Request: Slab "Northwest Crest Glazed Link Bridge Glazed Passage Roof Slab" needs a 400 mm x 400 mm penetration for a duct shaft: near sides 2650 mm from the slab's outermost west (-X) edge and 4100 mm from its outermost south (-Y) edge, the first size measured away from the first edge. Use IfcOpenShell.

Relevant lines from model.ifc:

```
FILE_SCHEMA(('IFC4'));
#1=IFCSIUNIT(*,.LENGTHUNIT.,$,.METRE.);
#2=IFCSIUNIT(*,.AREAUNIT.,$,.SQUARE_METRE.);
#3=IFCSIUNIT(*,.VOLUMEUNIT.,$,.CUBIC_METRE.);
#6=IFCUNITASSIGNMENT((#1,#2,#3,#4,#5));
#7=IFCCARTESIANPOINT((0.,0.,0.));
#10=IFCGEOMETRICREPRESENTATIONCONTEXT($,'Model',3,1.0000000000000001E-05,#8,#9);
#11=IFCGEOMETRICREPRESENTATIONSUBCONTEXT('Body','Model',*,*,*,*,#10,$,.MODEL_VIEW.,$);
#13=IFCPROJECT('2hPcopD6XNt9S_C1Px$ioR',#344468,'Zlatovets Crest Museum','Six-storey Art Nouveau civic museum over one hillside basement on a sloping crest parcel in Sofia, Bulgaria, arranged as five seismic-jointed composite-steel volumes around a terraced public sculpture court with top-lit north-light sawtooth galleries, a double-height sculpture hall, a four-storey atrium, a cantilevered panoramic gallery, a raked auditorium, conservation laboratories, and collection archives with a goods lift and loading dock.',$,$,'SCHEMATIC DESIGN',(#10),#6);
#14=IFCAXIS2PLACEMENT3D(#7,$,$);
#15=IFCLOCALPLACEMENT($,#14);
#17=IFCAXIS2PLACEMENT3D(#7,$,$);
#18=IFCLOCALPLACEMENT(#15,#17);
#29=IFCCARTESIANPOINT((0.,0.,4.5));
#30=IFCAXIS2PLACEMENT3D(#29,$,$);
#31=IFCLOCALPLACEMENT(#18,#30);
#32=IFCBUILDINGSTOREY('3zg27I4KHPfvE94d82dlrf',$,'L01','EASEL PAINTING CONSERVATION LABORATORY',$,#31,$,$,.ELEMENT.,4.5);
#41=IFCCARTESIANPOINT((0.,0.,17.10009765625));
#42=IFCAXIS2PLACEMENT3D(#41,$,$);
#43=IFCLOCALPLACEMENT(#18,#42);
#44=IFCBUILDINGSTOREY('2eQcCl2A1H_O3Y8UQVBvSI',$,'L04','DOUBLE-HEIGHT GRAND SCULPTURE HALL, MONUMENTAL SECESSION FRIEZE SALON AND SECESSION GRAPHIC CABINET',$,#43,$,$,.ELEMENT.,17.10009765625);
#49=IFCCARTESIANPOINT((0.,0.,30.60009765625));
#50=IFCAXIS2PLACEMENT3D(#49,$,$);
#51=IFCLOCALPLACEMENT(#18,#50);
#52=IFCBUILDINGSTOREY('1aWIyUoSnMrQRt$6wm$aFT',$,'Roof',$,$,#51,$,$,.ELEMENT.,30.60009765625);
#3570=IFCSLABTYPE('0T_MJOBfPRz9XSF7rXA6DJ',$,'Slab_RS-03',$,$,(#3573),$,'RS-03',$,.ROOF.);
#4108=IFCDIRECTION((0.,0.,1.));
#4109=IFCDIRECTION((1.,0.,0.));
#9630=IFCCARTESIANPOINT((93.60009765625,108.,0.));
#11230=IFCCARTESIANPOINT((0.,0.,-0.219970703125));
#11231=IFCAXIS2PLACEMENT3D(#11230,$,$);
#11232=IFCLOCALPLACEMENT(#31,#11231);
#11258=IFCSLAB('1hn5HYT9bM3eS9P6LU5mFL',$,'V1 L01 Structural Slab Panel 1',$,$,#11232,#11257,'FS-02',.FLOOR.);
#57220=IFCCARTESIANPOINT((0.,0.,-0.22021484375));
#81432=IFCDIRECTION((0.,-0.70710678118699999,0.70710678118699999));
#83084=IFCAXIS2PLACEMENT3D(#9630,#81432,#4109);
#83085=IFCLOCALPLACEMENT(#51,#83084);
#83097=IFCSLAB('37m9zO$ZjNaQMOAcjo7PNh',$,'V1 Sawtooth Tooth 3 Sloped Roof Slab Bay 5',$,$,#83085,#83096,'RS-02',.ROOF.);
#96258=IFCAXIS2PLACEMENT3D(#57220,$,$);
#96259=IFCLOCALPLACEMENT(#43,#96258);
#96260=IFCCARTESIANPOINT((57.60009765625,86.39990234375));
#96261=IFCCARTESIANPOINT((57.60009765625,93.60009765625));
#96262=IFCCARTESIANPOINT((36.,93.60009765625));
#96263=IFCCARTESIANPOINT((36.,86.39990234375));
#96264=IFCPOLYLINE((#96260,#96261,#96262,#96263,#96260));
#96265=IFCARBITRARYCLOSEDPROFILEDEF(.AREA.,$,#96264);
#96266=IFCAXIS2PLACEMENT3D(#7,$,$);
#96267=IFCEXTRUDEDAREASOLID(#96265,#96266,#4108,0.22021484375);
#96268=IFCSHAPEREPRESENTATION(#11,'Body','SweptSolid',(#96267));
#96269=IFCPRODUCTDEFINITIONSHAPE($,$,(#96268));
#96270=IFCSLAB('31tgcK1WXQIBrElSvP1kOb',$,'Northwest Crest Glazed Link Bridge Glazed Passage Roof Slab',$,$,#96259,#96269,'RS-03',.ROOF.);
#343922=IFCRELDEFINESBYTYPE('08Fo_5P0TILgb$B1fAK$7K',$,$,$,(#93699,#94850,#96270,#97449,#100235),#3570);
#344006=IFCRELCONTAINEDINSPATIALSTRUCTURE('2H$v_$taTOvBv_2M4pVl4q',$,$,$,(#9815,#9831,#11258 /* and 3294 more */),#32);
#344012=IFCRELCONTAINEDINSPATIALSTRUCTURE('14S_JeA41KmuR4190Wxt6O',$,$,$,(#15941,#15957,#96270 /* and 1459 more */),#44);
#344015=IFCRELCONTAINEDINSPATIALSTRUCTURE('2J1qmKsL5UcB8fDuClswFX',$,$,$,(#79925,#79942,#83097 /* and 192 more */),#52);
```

```python
import numpy as np
import ifcopenshell
import ifcopenshell.api.feature
import ifcopenshell.api.geometry
import ifcopenshell.api.root
import ifcopenshell.geom
import ifcopenshell.util.placement
import ifcopenshell.util.representation
import ifcopenshell.util.shape
import ifcopenshell.util.unit

model = ifcopenshell.open("model.ifc")
unit_scale = ifcopenshell.util.unit.calculate_unit_scale(model)
settings = ifcopenshell.geom.settings()


def volume(element):
    """Net volume in cubic metres, openings subtracted."""
    shape = ifcopenshell.geom.create_shape(settings, element)
    return ifcopenshell.util.shape.get_volume(shape.geometry)


slab = model.by_guid("31tgcK1WXQIBrElSvP1kOb")
before = volume(slab)

# Extent in the slab's own axes, in metres. The edges named are its -X and -Y sides.
slab_shape = ifcopenshell.geom.create_shape(settings, slab)
vertices = ifcopenshell.util.shape.get_vertices(slab_shape.geometry)
x_min, y_min, bottom = vertices.min(axis=0)
top = vertices[:, 2].max()

opening = ifcopenshell.api.root.create_entity(model, ifc_class="IfcOpeningElement", name="Duct shaft opening", predefined_type="OPENING")
context = ifcopenshell.util.representation.get_context(model, "Model", "Body", "MODEL_VIEW")
width, depth = 0.4, 0.4
outline = [(0.0, 0.0), (width, 0.0), (width, depth), (0.0, depth), (0.0, 0.0)]
# Overshoot both faces by 50 mm so the cut is clean.
shape = ifcopenshell.api.geometry.add_slab_representation(
    model, context=context, depth=top - bottom + 0.1, polyline=outline
)
ifcopenshell.api.geometry.assign_representation(model, product=opening, representation=shape)

matrix = ifcopenshell.util.placement.get_local_placement(slab.ObjectPlacement)
matrix[:, 3] = matrix @ np.append(np.array([x_min + 2.65, y_min + 4.1, bottom - 0.05]) / unit_scale, 1.0)
ifcopenshell.api.geometry.edit_object_placement(model, product=opening, matrix=matrix, is_si=False)
ifcopenshell.api.feature.add_feature(model, feature=opening, element=slab)

after = volume(slab)

print(f"slab volume {before:.3f} -> {after:.3f} m3")

model.write("model-out.ifc")
```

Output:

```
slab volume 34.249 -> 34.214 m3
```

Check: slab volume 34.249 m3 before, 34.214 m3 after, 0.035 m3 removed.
